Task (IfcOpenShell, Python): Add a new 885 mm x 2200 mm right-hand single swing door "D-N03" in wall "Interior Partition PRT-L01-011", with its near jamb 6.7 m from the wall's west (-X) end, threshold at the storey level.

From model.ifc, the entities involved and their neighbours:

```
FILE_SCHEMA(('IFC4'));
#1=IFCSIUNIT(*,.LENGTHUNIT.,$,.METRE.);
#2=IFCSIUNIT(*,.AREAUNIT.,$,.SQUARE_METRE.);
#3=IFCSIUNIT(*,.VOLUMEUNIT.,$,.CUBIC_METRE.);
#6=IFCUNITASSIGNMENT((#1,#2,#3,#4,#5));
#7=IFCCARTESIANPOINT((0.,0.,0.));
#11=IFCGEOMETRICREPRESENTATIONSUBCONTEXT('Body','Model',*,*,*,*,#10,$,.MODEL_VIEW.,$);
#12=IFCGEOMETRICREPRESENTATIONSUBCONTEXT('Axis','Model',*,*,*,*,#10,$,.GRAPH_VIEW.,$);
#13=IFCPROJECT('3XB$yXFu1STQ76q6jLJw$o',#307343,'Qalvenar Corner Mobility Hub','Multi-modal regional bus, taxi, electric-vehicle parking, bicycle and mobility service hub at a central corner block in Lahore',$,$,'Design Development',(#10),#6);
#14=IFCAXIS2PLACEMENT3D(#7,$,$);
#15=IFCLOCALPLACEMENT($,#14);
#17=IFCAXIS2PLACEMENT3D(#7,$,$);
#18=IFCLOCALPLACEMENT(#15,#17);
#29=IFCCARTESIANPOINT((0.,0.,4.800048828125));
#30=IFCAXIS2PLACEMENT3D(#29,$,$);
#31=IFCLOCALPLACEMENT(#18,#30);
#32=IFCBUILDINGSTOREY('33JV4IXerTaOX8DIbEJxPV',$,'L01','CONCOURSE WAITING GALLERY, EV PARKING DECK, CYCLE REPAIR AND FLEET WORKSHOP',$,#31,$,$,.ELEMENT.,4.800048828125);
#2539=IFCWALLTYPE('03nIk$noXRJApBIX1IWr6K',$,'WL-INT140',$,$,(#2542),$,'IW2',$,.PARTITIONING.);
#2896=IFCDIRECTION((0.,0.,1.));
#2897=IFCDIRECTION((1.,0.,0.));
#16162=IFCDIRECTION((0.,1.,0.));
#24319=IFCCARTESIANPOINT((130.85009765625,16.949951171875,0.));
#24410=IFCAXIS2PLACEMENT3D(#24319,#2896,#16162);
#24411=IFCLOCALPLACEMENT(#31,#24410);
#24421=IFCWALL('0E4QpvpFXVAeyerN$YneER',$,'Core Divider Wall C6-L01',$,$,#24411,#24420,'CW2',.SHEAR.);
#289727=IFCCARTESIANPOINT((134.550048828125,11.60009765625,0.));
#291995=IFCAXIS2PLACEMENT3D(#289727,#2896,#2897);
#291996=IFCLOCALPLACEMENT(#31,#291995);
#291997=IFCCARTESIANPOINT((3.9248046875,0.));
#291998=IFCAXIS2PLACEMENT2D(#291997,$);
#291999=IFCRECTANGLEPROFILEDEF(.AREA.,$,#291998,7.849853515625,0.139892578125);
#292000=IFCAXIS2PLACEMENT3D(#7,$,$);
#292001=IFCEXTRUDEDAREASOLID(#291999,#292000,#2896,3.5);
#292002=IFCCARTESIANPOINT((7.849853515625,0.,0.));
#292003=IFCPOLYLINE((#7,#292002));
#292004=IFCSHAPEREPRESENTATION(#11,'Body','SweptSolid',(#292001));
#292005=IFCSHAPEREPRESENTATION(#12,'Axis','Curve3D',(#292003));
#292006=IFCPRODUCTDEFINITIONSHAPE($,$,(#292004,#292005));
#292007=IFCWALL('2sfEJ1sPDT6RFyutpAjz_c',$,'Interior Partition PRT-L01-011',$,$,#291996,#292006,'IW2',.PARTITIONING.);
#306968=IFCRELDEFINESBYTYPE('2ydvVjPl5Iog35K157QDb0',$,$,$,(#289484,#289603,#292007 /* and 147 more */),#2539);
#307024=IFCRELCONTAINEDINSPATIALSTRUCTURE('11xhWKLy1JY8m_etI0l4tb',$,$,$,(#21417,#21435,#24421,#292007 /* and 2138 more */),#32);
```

```python
import numpy as np
import ifcopenshell
import ifcopenshell.api.feature
import ifcopenshell.api.geometry
import ifcopenshell.api.root
import ifcopenshell.api.spatial
import ifcopenshell.geom
import ifcopenshell.util.element
import ifcopenshell.util.placement
import ifcopenshell.util.representation
import ifcopenshell.util.shape
import ifcopenshell.util.unit

model = ifcopenshell.open("model.ifc")
unit_scale = ifcopenshell.util.unit.calculate_unit_scale(model)
settings = ifcopenshell.geom.settings()


def volume(element):
    """Net volume in cubic metres, openings subtracted."""
    shape = ifcopenshell.geom.create_shape(settings, element)
    return ifcopenshell.util.shape.get_volume(shape.geometry)


wall = model.by_guid("2sfEJ1sPDT6RFyutpAjz_c")
storey = ifcopenshell.util.element.get_container(wall, ifc_class="IfcBuildingStorey")
context = ifcopenshell.util.representation.get_context(model, "Model", "Body", "MODEL_VIEW")
before = volume(wall)

width, height, from_end, sill = 0.885, 2.2, 6.7, 0.0  # metres

# The wall runs along its own X axis, and the end named is its -X end.
wall_shape = ifcopenshell.geom.create_shape(settings, wall)
x, y, z = ifcopenshell.util.shape.get_vertices(wall_shape.geometry).T
start = x.min() + from_end
face, thickness = float(y.min()), float(y.max() - y.min())
wall_matrix = ifcopenshell.util.placement.get_local_placement(wall.ObjectPlacement)
level = ifcopenshell.util.placement.get_local_placement(storey.ObjectPlacement)[2, 3]


def in_wall(x, y):
    """Placement at x, y metres in the wall's axes, at sill height."""
    matrix = wall_matrix.copy()
    matrix[:, 3] = wall_matrix @ np.array([x / unit_scale, y / unit_scale, 0.0, 1.0])
    matrix[2, 3] = level + sill / unit_scale
    return matrix


# Opening: a box that overshoots both wall faces by 50 mm.
opening = ifcopenshell.api.root.create_entity(model, ifc_class="IfcOpeningElement", predefined_type="OPENING")
box = ifcopenshell.api.geometry.add_wall_representation(
    model, context=context, length=width, height=height, thickness=thickness + 0.1
)
ifcopenshell.api.geometry.assign_representation(model, product=opening, representation=box)
ifcopenshell.api.geometry.edit_object_placement(model, product=opening, matrix=in_wall(start, face - 0.05), is_si=False)
ifcopenshell.api.feature.add_feature(model, feature=opening, element=wall)

door = ifcopenshell.api.root.create_entity(model, ifc_class="IfcDoor", name="D-N03", predefined_type="DOOR")
door.OverallWidth, door.OverallHeight = width / unit_scale, height / unit_scale
door.OperationType = "SINGLE_SWING_RIGHT"
body = ifcopenshell.api.geometry.add_door_representation(
    model,
    context=context,
    overall_width=door.OverallWidth,
    overall_height=door.OverallHeight,
    operation_type="SINGLE_SWING_RIGHT",
    lining_properties={"LiningDepth": thickness / unit_scale, "ThresholdDepth": thickness / unit_scale},
)
ifcopenshell.api.geometry.assign_representation(model, product=door, representation=body)
ifcopenshell.api.spatial.assign_container(model, products=[door], relating_structure=storey)
ifcopenshell.api.feature.add_filling(model, opening=opening, element=door)

# The lining spans the wall, so the door starts at the wall face.
ifcopenshell.api.geometry.edit_object_placement(model, product=door, matrix=in_wall(start, face), is_si=False)

after = volume(wall)

print(f"wall volume {before:.3f} -> {after:.3f} m3")

model.write("model_v2.ifc")
```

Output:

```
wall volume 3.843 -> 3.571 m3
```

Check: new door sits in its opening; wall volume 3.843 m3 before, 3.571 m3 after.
